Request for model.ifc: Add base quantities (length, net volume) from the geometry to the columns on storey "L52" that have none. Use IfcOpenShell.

First a look at what the model holds.

```python
import ifcopenshell
import ifcopenshell.util.element
import ifcopenshell.util.unit

model = ifcopenshell.open("model.ifc")
print(model.schema)
for unit_type in ("LENGTHUNIT", "AREAUNIT", "VOLUMEUNIT"):
    print(unit_type, ifcopenshell.util.unit.calculate_unit_scale(model, unit_type))
storey = next(s for s in model.by_type("IfcBuildingStorey") if s.Name == "L52")
columns = [e for e in ifcopenshell.util.element.get_decomposition(storey) if e.is_a("IfcColumn")]
for e in sorted(columns, key=lambda e: e.id()):
    print(e.id(), e.is_a(), e.Name, list(ifcopenshell.util.element.get_psets(e, qtos_only=True)), sep=" | ")
```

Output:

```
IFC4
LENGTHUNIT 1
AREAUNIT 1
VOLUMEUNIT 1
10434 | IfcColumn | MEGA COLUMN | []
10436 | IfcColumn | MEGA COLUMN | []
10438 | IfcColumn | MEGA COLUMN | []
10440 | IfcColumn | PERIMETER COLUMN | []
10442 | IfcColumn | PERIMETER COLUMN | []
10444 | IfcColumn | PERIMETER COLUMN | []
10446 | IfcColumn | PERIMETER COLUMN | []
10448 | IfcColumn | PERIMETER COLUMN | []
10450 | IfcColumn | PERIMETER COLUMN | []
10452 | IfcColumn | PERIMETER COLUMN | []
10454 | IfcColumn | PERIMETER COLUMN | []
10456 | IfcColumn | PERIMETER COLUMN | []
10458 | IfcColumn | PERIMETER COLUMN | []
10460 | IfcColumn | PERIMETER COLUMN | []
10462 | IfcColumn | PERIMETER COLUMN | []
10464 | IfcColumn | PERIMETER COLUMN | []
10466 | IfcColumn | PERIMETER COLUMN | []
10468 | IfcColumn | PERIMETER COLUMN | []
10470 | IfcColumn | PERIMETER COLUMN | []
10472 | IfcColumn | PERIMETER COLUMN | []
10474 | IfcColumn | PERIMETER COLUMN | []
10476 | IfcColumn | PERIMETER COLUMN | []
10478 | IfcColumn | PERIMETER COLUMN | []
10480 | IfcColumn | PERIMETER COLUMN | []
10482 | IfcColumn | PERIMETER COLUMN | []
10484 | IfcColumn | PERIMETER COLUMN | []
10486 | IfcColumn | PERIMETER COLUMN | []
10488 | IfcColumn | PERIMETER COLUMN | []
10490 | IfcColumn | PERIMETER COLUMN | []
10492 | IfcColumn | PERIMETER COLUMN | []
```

```python
import ifcopenshell
import ifcopenshell.api.pset
import ifcopenshell.geom
import ifcopenshell.util.element
import ifcopenshell.util.shape
import ifcopenshell.util.unit

model = ifcopenshell.open("model.ifc")
unit_scale = ifcopenshell.util.unit.calculate_unit_scale(model)
volume_scale = ifcopenshell.util.unit.calculate_unit_scale(model, "VOLUMEUNIT")
settings = ifcopenshell.geom.settings()

storey = next(s for s in model.by_type("IfcBuildingStorey") if s.Name == "L52")
columns = [e for e in ifcopenshell.util.element.get_decomposition(storey) if e.is_a("IfcColumn")]

for e in sorted(columns, key=lambda e: e.id()):
    if ifcopenshell.util.element.get_psets(e, qtos_only=True, should_inherit=False):
        continue
    # Geometry comes back in metres, in the element's own axes.
    shape = ifcopenshell.geom.create_shape(settings, e)
    values = {
        "Length": ifcopenshell.util.shape.get_z(shape.geometry) / unit_scale,
        "NetVolume": ifcopenshell.util.shape.get_volume(shape.geometry) / volume_scale,
    }
    qto = ifcopenshell.api.pset.add_qto(model, product=e, name="Qto_ColumnBaseQuantities")
    ifcopenshell.api.pset.edit_qto(model, qto=qto, properties=values)
    print(e.id(), {k: round(v, 3) for k, v in values.items()})

model.write("model_updated.ifc")
```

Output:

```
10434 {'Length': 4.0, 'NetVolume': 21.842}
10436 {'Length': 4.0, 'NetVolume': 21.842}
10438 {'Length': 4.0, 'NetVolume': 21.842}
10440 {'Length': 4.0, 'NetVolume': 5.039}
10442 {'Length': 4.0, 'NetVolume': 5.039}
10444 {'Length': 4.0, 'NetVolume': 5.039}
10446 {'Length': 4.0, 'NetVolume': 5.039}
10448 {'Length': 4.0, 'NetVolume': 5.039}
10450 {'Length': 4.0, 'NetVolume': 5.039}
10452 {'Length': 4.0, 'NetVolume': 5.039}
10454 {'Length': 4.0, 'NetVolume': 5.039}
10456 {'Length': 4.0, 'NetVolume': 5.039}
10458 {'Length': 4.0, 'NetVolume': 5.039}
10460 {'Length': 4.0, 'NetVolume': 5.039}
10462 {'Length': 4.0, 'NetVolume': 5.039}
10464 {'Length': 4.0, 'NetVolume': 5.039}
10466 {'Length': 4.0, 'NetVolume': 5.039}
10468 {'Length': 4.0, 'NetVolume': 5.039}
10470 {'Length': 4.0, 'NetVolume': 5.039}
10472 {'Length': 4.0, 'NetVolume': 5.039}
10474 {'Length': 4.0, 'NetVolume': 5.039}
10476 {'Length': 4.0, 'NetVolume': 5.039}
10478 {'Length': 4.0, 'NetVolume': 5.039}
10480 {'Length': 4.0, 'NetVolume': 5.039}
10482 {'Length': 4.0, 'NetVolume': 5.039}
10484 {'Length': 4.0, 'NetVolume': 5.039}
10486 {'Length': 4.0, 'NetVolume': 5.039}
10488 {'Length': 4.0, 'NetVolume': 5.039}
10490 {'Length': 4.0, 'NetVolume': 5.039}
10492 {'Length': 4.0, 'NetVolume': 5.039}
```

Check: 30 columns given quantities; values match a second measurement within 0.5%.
